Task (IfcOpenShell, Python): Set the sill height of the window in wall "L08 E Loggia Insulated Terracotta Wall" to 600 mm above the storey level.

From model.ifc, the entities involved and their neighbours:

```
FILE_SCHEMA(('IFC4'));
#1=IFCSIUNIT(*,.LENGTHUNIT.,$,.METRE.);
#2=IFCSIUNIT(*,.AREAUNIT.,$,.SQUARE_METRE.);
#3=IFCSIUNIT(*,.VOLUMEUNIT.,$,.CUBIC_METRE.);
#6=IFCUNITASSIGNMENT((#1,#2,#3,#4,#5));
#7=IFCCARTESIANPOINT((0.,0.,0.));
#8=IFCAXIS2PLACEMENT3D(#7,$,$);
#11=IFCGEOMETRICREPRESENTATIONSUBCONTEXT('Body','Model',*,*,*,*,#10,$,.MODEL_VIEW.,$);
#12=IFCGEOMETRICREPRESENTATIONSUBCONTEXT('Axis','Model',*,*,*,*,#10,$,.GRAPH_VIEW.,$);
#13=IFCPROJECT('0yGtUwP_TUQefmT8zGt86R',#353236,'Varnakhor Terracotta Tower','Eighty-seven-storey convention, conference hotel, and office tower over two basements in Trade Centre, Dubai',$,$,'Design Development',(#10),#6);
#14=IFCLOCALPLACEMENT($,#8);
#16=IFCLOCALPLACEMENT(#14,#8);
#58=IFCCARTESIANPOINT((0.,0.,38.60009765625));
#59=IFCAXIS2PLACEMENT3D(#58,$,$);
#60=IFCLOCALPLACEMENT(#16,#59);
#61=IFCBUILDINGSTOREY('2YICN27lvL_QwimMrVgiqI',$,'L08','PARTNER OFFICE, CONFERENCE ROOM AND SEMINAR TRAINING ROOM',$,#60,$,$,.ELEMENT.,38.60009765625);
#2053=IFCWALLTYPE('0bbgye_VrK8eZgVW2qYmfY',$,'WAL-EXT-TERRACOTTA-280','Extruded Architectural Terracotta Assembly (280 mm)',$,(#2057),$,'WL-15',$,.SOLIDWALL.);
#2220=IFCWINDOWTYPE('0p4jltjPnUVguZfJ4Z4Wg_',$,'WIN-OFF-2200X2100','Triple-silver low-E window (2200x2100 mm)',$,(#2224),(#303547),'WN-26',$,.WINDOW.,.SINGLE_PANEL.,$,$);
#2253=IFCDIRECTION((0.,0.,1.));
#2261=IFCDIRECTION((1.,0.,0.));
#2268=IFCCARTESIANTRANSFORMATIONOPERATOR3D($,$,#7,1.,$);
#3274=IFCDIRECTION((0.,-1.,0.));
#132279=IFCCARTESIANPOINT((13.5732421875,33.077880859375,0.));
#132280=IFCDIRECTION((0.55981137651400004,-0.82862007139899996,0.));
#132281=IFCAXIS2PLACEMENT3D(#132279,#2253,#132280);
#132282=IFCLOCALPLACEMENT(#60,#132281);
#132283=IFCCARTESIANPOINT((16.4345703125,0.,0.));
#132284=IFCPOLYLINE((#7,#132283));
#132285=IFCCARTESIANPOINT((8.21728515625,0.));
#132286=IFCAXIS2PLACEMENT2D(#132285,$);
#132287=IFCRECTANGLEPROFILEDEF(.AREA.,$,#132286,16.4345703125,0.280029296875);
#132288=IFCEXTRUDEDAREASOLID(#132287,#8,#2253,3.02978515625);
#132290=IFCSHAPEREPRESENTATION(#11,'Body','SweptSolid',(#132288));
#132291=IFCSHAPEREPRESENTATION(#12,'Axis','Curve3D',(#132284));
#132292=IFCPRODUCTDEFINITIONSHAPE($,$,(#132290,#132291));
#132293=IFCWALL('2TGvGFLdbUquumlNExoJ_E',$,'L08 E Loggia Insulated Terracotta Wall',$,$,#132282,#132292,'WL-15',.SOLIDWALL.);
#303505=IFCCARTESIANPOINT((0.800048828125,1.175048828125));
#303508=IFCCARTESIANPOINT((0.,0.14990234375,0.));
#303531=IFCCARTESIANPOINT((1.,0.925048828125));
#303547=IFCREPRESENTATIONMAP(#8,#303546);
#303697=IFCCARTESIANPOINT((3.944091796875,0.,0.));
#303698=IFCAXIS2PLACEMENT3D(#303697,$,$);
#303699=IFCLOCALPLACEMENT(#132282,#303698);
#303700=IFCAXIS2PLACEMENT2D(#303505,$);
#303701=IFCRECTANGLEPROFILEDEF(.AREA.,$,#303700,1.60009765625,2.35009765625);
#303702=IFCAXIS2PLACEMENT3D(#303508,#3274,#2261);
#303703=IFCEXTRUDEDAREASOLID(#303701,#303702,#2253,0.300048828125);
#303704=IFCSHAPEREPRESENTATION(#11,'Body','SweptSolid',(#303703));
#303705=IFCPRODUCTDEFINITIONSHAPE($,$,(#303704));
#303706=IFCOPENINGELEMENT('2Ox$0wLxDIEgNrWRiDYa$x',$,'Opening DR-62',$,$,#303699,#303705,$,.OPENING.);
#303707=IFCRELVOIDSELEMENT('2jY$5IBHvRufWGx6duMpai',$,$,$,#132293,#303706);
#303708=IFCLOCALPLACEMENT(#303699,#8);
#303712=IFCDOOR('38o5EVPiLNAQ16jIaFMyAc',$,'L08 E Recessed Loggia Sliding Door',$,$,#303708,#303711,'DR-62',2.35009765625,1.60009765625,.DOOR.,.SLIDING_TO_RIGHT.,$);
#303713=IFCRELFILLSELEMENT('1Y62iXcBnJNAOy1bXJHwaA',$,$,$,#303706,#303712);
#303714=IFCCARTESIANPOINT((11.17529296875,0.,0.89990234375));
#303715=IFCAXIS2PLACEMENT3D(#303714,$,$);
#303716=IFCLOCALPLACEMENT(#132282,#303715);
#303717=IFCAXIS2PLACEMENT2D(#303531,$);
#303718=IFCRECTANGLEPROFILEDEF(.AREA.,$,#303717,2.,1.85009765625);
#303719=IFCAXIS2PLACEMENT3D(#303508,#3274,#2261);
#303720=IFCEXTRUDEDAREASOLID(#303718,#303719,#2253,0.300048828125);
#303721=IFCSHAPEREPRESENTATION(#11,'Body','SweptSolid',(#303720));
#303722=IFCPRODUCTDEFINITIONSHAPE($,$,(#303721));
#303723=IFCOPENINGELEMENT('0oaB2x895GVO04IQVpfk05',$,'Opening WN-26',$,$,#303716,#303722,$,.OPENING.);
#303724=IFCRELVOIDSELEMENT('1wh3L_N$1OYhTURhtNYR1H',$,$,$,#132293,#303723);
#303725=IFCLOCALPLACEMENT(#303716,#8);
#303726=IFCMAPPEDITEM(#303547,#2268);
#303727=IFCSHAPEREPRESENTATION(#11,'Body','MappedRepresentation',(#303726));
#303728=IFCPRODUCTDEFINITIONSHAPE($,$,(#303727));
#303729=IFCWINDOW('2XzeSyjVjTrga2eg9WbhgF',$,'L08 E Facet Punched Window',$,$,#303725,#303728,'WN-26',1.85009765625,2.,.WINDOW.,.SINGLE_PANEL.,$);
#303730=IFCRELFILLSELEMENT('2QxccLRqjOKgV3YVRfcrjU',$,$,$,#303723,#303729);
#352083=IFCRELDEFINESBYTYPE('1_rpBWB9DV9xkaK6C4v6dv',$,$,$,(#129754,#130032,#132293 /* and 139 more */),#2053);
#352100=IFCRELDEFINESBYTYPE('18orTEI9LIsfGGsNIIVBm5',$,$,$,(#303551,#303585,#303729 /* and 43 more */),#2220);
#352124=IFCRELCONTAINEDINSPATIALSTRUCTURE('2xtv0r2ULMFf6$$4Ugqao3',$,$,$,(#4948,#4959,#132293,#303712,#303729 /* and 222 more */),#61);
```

```python
import numpy as np
import ifcopenshell
import ifcopenshell.api.geometry
import ifcopenshell.geom
import ifcopenshell.util.element
import ifcopenshell.util.placement
import ifcopenshell.util.shape
import ifcopenshell.util.unit

model = ifcopenshell.open("model.ifc")
unit_scale = ifcopenshell.util.unit.calculate_unit_scale(model)

window = model.by_guid("2XzeSyjVjTrga2eg9WbhgF")
opening = window.FillsVoids[0].RelatingOpeningElement
storey = ifcopenshell.util.element.get_container(window, ifc_class="IfcBuildingStorey")
level = ifcopenshell.util.placement.get_local_placement(storey.ObjectPlacement)[2, 3]

# The opening's origin need not be at the sill, so measure its lowest point.
shape = ifcopenshell.geom.create_shape(ifcopenshell.geom.settings(), opening)
bottom = ifcopenshell.util.shape.get_shape_bottom_elevation(shape, shape.geometry) / unit_scale
dz = level + 0.6 / unit_scale - bottom

shift = np.array([0.0, 0.0, dz])
# The window is placed relative to its opening, so it follows when the opening moves.
matrix = ifcopenshell.util.placement.get_local_placement(opening.ObjectPlacement)
matrix[:3, 3] += shift
ifcopenshell.api.geometry.edit_object_placement(
    model, product=opening, matrix=matrix, is_si=False, should_transform_children=True
)

print(f"moved by {dz * unit_scale:+.3f} m")

model.write("model_rev.ifc")
```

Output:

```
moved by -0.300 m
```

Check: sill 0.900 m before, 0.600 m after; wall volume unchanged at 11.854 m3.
